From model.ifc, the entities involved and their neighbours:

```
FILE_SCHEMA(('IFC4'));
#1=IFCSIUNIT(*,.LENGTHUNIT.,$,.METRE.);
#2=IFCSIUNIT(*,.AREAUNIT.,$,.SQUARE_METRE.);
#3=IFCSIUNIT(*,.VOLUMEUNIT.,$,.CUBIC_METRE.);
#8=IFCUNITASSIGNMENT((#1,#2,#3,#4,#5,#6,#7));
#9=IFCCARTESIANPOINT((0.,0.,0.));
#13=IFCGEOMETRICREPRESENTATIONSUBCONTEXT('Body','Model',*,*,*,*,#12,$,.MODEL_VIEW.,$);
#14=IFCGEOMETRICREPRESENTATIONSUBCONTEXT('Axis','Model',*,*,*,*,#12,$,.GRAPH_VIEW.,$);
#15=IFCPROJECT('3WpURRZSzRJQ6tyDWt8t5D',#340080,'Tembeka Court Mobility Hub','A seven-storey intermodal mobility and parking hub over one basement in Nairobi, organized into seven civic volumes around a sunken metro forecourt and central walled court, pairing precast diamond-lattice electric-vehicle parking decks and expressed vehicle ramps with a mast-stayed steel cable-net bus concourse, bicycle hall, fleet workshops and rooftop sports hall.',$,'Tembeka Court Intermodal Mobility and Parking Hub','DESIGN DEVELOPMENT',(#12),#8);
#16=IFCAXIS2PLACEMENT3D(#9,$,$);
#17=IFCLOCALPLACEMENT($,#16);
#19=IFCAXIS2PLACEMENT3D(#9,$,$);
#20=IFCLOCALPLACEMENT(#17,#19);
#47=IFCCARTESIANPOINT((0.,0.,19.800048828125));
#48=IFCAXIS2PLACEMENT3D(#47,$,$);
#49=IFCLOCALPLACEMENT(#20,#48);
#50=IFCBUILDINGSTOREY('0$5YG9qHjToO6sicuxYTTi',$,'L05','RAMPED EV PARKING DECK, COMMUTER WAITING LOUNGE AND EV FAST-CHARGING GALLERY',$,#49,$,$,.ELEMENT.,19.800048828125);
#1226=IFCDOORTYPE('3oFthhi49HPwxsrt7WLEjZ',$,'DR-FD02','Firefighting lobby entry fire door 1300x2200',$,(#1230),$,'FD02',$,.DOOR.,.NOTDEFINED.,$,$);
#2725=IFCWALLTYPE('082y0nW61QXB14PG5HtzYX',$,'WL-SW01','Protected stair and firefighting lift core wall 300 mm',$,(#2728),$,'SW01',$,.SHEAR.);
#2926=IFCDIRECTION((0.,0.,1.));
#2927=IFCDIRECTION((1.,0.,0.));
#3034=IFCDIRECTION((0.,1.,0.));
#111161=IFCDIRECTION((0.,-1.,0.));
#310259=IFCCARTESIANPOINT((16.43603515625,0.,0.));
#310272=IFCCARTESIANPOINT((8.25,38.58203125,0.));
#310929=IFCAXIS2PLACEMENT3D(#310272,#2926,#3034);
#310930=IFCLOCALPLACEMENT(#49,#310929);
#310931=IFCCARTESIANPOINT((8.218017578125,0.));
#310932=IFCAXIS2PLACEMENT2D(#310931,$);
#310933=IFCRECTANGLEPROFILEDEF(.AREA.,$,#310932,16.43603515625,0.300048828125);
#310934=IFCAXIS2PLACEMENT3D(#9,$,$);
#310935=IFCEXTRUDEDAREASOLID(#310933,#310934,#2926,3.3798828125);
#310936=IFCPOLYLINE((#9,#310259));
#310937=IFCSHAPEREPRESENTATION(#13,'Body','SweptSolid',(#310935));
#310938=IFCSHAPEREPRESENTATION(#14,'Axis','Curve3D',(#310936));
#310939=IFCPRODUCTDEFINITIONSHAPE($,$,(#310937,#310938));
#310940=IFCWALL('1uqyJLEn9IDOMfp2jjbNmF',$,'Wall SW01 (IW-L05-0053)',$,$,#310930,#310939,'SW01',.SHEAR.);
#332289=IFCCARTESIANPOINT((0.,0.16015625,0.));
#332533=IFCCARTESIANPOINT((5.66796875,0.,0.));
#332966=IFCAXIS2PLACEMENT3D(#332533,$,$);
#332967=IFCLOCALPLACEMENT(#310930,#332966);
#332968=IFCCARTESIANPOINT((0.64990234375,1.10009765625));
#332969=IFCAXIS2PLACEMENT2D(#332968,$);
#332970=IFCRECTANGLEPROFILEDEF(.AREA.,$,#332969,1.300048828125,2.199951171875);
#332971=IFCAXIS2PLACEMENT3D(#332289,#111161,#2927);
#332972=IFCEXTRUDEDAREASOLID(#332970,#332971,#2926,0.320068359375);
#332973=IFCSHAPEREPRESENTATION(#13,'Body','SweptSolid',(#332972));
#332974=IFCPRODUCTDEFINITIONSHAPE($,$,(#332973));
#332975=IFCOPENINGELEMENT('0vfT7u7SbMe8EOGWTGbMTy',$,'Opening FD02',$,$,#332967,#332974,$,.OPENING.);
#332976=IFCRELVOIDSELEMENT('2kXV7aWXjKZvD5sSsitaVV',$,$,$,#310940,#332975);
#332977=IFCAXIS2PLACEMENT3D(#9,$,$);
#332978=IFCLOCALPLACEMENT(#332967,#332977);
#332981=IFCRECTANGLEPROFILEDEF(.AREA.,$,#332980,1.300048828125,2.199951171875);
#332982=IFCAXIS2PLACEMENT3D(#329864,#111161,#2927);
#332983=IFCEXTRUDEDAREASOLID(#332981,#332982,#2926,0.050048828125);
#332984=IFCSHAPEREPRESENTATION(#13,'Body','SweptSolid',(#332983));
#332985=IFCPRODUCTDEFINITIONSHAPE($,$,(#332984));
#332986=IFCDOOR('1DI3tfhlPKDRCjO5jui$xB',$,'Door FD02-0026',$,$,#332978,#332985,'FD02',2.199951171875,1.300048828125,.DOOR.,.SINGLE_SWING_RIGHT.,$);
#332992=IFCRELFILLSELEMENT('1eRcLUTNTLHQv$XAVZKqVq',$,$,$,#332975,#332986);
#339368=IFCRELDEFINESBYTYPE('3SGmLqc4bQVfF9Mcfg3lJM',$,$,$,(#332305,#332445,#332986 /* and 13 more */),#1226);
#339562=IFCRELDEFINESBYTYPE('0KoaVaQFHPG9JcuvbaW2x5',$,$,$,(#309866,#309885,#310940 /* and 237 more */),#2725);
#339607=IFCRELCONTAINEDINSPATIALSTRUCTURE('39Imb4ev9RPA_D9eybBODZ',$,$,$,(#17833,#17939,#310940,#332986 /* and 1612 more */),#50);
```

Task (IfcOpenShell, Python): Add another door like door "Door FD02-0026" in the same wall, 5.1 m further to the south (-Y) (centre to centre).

```python
import ifcopenshell
import ifcopenshell.api.feature
import ifcopenshell.api.geometry
import ifcopenshell.api.root
import ifcopenshell.geom
import ifcopenshell.util.element
import ifcopenshell.util.placement
import ifcopenshell.util.shape
import ifcopenshell.util.unit

model = ifcopenshell.open("model.ifc")
unit_scale = ifcopenshell.util.unit.calculate_unit_scale(model)
settings = ifcopenshell.geom.settings()


def volume(element):
    """Net volume in cubic metres, openings subtracted."""
    shape = ifcopenshell.geom.create_shape(settings, element)
    return ifcopenshell.util.shape.get_volume(shape.geometry)


door = model.by_guid("1DI3tfhlPKDRCjO5jui$xB")
opening = door.FillsVoids[0].RelatingOpeningElement
wall = opening.VoidsElements[0].RelatingBuildingElement
before = volume(wall)
shift = ifcopenshell.util.placement.get_local_placement(wall.ObjectPlacement)[:3, 0] * -5.1 / unit_scale

# copy_class copies the void relationship, type, container and properties, but no geometry.
new_opening = ifcopenshell.api.root.copy_class(model, product=opening)
new_opening.Representation = ifcopenshell.util.element.copy_deep(
    model, opening.Representation, exclude=["IfcGeometricRepresentationContext", "IfcRepresentationMap"]
)
new_door = ifcopenshell.api.root.copy_class(model, product=door)
new_door.Representation = ifcopenshell.util.element.copy_deep(
    model, door.Representation, exclude=["IfcGeometricRepresentationContext", "IfcRepresentationMap"]
)
new_door.Tag = None
ifcopenshell.api.feature.add_filling(model, opening=new_opening, element=new_door)

for old, new in ((opening, new_opening), (door, new_door)):
    matrix = ifcopenshell.util.placement.get_local_placement(old.ObjectPlacement)
    matrix[:3, 3] += shift
    ifcopenshell.api.geometry.edit_object_placement(model, product=new, matrix=matrix, is_si=False)

after = volume(wall)

print(f"wall volume {before:.3f} -> {after:.3f} m3")

model.write("model_updated.ifc")
```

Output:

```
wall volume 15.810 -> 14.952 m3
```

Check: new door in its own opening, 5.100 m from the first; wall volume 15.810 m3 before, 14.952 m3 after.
